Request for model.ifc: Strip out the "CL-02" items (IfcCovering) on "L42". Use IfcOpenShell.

First a look at what the model holds.

```python
import ifcopenshell
import ifcopenshell.util.element

model = ifcopenshell.open("model.ifc")
print(model.schema)
storey = next(s for s in model.by_type("IfcBuildingStorey") if s.Name == "L42")
coverings = [e for e in ifcopenshell.util.element.get_decomposition(storey) if e.is_a("IfcCovering")]
seen = {}
for e in coverings:
    element_type = ifcopenshell.util.element.get_type(e)
    name = element_type.Name if element_type not in (None, e) else None
    seen[name] = seen.get(name, 0) + 1
for name, count in sorted(seen.items(), key=str):
    print(count, "x", name)
```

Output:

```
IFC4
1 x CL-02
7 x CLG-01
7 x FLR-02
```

```python
import ifcopenshell
import ifcopenshell.api.root
import ifcopenshell.util.element

model = ifcopenshell.open("model.ifc")

storey = next(s for s in model.by_type("IfcBuildingStorey") if s.Name == "L42")
coverings = [e for e in ifcopenshell.util.element.get_decomposition(storey) if e.is_a("IfcCovering")]
targets = [e for e in coverings if (t := ifcopenshell.util.element.get_type(e)) not in (None, e) and t.Name == "CL-02"]

for e in targets:
    ifcopenshell.api.root.remove_product(model, product=e)
print(len(targets), "removed")

model.write("model_rev.ifc")
```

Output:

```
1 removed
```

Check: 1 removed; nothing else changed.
